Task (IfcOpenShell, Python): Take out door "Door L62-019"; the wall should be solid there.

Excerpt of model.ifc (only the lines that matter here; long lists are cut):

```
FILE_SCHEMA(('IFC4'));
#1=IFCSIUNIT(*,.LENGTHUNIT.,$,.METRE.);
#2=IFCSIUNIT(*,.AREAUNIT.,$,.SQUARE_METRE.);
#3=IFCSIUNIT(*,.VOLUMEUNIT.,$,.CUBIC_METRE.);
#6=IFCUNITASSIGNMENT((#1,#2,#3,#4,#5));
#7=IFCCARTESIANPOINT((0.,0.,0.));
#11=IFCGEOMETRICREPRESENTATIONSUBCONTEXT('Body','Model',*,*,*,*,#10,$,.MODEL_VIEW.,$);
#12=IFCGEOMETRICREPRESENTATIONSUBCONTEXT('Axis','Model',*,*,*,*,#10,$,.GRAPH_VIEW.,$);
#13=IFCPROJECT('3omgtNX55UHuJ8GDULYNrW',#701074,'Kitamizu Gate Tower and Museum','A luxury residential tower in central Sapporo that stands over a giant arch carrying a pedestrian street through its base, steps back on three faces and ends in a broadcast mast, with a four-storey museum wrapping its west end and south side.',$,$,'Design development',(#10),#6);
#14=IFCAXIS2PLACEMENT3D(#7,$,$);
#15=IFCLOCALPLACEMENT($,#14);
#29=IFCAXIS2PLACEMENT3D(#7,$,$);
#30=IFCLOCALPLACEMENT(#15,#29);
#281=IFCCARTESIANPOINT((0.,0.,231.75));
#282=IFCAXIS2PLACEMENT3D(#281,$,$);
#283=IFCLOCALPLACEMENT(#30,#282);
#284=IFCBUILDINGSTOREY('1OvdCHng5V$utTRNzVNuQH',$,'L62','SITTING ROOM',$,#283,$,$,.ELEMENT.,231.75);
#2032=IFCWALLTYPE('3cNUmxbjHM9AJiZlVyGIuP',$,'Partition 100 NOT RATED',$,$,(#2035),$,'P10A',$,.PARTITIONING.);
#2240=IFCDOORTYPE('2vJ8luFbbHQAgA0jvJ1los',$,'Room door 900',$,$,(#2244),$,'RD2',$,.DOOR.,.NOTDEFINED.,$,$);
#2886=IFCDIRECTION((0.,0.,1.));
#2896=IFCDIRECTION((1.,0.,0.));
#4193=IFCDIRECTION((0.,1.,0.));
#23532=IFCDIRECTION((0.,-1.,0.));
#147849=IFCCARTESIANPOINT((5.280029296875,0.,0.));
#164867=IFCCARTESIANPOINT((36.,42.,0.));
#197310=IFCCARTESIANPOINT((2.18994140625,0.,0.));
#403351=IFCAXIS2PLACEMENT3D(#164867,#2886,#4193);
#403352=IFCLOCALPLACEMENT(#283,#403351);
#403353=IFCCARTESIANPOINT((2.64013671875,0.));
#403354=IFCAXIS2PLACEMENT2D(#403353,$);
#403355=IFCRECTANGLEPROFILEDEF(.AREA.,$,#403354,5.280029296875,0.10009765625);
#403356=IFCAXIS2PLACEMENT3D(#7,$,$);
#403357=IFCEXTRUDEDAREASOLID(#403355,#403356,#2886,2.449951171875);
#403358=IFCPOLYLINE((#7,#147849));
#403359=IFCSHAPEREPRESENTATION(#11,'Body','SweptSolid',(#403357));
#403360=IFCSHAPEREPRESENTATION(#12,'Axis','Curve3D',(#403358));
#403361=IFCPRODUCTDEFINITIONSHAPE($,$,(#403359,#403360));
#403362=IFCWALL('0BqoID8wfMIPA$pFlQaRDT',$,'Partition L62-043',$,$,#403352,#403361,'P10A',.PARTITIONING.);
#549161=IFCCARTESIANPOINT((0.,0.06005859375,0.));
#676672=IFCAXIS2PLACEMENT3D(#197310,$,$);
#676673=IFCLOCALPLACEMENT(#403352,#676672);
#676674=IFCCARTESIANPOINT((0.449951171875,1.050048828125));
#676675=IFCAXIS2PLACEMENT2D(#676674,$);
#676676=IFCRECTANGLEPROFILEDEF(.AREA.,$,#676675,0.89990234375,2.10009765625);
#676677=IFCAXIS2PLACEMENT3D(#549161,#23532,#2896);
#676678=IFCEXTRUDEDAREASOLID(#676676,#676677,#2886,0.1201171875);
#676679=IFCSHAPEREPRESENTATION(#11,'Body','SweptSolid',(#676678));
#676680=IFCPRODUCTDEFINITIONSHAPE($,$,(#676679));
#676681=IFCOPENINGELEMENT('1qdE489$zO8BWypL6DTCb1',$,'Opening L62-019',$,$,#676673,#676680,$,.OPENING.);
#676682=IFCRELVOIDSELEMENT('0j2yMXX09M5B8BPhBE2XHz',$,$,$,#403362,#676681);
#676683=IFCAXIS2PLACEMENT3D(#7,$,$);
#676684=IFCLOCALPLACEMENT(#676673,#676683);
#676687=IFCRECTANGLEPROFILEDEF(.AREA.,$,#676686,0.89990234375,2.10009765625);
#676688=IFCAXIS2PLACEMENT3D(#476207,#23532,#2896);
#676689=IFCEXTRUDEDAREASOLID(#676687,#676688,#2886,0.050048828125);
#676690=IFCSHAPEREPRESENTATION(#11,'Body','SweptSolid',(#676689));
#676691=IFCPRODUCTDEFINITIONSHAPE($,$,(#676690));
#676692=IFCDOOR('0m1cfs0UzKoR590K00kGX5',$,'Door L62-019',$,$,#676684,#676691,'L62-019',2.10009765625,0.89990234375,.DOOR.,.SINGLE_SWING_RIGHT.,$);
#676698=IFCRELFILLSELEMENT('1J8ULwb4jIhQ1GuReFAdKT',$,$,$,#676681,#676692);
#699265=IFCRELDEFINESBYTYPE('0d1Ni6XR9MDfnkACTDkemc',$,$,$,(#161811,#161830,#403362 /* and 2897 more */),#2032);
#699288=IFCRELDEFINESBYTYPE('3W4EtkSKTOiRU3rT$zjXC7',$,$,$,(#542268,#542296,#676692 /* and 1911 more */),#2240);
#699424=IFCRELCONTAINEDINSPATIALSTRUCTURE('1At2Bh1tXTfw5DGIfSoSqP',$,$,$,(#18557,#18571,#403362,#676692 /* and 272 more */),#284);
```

```python
import ifcopenshell
import ifcopenshell.api.feature
import ifcopenshell.api.root
import ifcopenshell.geom
import ifcopenshell.util.shape

model = ifcopenshell.open("model.ifc")
settings = ifcopenshell.geom.settings()


def volume(element):
    """Net volume in cubic metres, openings subtracted."""
    shape = ifcopenshell.geom.create_shape(settings, element)
    return ifcopenshell.util.shape.get_volume(shape.geometry)


door = model.by_id(676692)
opening = door.FillsVoids[0].RelatingOpeningElement
wall = opening.VoidsElements[0].RelatingBuildingElement
before = volume(wall)

ifcopenshell.api.root.remove_product(model, product=door)
ifcopenshell.api.feature.remove_feature(model, feature=opening)

after = volume(wall)

print(f"wall volume {before:.3f} -> {after:.3f} m3")

model.write("model-out.ifc")
```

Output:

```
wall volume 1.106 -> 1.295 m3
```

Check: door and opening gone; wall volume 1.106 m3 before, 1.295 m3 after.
